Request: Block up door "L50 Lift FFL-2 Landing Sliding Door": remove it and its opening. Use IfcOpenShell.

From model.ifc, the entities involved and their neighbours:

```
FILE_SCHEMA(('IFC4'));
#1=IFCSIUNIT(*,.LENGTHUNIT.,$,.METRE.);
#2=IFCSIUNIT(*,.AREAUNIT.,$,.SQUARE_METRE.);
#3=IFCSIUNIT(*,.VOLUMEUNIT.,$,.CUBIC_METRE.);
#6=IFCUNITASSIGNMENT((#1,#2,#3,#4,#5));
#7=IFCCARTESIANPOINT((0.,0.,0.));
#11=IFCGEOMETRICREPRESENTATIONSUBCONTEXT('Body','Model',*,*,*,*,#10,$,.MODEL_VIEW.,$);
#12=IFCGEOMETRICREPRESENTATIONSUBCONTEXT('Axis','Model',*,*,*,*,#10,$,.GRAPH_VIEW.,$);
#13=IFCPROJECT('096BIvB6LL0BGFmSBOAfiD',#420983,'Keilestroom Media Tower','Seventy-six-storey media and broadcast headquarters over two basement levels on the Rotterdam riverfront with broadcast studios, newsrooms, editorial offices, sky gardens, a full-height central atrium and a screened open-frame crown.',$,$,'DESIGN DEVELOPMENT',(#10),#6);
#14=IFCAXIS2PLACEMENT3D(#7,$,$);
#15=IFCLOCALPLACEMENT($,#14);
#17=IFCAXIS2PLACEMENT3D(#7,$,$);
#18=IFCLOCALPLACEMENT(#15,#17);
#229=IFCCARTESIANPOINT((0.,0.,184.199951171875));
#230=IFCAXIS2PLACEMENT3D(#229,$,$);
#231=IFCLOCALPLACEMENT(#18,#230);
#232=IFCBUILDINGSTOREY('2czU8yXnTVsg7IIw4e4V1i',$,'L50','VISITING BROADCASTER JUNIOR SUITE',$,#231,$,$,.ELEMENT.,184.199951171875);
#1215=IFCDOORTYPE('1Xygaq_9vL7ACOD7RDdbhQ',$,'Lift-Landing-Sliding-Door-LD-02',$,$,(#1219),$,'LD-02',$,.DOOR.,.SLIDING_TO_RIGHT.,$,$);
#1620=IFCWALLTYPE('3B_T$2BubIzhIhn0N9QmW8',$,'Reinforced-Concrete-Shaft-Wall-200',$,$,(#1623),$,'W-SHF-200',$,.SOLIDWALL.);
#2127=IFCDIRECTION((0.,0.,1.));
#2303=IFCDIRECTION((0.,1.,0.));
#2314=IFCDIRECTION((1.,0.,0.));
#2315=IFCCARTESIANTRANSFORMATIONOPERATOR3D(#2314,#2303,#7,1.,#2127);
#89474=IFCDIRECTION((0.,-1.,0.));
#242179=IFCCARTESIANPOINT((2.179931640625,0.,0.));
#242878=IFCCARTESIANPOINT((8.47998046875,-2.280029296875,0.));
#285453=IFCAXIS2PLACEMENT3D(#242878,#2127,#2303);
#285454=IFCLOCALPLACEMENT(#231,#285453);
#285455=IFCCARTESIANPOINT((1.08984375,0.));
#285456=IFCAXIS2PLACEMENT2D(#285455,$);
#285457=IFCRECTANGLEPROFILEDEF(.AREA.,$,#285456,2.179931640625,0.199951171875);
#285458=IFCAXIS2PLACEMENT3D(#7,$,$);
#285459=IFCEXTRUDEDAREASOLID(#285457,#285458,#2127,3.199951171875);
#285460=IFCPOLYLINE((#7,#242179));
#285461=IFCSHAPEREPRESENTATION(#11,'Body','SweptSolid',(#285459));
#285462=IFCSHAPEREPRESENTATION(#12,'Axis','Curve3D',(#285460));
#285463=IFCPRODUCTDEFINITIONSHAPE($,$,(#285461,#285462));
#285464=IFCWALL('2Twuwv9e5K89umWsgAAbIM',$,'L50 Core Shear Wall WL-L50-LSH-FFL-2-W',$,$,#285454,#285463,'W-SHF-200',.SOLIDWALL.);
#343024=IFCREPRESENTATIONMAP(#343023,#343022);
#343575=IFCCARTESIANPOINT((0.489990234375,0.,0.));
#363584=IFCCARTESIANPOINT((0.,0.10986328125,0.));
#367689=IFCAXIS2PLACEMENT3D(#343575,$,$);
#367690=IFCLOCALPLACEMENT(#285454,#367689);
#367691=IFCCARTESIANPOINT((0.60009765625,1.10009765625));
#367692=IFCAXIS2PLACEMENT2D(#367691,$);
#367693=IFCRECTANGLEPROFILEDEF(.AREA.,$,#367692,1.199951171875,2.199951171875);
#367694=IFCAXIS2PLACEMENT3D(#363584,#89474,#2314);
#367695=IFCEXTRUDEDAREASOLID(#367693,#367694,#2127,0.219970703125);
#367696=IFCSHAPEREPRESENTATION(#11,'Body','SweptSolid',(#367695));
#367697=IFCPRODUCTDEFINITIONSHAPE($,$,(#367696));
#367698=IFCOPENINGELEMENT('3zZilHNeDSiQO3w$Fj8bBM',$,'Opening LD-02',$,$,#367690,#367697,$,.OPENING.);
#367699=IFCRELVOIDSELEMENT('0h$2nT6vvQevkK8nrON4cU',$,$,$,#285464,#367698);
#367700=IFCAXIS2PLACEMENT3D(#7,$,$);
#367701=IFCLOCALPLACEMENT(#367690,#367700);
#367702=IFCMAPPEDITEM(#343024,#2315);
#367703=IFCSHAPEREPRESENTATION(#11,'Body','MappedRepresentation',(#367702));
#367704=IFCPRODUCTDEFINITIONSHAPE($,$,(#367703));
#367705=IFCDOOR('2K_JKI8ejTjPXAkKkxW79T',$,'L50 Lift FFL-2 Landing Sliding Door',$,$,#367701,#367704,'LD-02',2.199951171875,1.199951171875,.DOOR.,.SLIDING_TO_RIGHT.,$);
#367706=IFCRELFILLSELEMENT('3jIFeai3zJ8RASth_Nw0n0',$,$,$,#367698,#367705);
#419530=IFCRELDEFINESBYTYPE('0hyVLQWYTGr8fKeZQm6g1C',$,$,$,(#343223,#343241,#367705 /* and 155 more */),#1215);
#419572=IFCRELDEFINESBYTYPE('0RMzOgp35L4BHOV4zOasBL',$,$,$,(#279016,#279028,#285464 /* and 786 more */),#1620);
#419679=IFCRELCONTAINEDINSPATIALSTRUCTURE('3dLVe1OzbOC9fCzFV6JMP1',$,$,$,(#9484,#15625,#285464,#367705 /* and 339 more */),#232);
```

```python
import ifcopenshell
import ifcopenshell.api.feature
import ifcopenshell.api.root
import ifcopenshell.geom
import ifcopenshell.util.shape

model = ifcopenshell.open("model.ifc")
settings = ifcopenshell.geom.settings()


def volume(element):
    """Net volume in cubic metres, openings subtracted."""
    shape = ifcopenshell.geom.create_shape(settings, element)
    return ifcopenshell.util.shape.get_volume(shape.geometry)


door = model.by_guid("2K_JKI8ejTjPXAkKkxW79T")
opening = door.FillsVoids[0].RelatingOpeningElement
wall = opening.VoidsElements[0].RelatingBuildingElement
before = volume(wall)

ifcopenshell.api.root.remove_product(model, product=door)
ifcopenshell.api.feature.remove_feature(model, feature=opening)

after = volume(wall)

print(f"wall volume {before:.3f} -> {after:.3f} m3")

model.write("model_v2.ifc")
```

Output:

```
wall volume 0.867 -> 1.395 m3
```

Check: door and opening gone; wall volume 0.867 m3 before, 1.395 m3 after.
